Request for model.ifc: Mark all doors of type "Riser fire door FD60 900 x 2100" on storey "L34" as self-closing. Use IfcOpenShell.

First a look at what the model holds.

```python
import ifcopenshell
import ifcopenshell.util.element

model = ifcopenshell.open("model.ifc")
print(model.schema)
storey = next(s for s in model.by_type("IfcBuildingStorey") if s.Name == "L34")
doors = [e for e in ifcopenshell.util.element.get_decomposition(storey) if e.is_a("IfcDoor")]
seen = {}
for e in doors:
    element_type = ifcopenshell.util.element.get_type(e)
    key = (element_type.Name if element_type != e and element_type else None, ifcopenshell.util.element.get_pset(e, "Pset_DoorCommon", "SelfClosing"))
    seen[key] = seen.get(key, 0) + 1
for (name, value), count in sorted(seen.items(), key=str):
    print(count, "x", name, "|", value)
```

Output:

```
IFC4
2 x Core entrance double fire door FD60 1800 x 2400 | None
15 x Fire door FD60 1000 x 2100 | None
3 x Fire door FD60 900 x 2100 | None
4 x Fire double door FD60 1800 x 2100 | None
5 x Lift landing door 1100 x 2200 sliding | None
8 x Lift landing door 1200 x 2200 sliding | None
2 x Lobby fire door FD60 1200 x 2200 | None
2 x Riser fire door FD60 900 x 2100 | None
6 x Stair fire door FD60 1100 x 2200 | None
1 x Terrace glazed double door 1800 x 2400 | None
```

```python
import ifcopenshell
import ifcopenshell.api.pset
import ifcopenshell.util.element

model = ifcopenshell.open("model.ifc")

storey = next(s for s in model.by_type("IfcBuildingStorey") if s.Name == "L34")
doors = [e for e in ifcopenshell.util.element.get_decomposition(storey) if e.is_a("IfcDoor")]

count = 0
for e in doors:
    element_type = ifcopenshell.util.element.get_type(e)
    if element_type in (None, e) or element_type.Name != "Riser fire door FD60 900 x 2100":
        continue
    # add_pset returns the element's existing set when there is one.
    pset = ifcopenshell.api.pset.add_pset(model, product=e, name="Pset_DoorCommon")
    ifcopenshell.api.pset.edit_pset(model, pset=pset, properties={"SelfClosing": True})
    count += 1

print(count, "doors updated")

model.write("model_rev.ifc")
```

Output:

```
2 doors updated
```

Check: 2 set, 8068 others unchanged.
